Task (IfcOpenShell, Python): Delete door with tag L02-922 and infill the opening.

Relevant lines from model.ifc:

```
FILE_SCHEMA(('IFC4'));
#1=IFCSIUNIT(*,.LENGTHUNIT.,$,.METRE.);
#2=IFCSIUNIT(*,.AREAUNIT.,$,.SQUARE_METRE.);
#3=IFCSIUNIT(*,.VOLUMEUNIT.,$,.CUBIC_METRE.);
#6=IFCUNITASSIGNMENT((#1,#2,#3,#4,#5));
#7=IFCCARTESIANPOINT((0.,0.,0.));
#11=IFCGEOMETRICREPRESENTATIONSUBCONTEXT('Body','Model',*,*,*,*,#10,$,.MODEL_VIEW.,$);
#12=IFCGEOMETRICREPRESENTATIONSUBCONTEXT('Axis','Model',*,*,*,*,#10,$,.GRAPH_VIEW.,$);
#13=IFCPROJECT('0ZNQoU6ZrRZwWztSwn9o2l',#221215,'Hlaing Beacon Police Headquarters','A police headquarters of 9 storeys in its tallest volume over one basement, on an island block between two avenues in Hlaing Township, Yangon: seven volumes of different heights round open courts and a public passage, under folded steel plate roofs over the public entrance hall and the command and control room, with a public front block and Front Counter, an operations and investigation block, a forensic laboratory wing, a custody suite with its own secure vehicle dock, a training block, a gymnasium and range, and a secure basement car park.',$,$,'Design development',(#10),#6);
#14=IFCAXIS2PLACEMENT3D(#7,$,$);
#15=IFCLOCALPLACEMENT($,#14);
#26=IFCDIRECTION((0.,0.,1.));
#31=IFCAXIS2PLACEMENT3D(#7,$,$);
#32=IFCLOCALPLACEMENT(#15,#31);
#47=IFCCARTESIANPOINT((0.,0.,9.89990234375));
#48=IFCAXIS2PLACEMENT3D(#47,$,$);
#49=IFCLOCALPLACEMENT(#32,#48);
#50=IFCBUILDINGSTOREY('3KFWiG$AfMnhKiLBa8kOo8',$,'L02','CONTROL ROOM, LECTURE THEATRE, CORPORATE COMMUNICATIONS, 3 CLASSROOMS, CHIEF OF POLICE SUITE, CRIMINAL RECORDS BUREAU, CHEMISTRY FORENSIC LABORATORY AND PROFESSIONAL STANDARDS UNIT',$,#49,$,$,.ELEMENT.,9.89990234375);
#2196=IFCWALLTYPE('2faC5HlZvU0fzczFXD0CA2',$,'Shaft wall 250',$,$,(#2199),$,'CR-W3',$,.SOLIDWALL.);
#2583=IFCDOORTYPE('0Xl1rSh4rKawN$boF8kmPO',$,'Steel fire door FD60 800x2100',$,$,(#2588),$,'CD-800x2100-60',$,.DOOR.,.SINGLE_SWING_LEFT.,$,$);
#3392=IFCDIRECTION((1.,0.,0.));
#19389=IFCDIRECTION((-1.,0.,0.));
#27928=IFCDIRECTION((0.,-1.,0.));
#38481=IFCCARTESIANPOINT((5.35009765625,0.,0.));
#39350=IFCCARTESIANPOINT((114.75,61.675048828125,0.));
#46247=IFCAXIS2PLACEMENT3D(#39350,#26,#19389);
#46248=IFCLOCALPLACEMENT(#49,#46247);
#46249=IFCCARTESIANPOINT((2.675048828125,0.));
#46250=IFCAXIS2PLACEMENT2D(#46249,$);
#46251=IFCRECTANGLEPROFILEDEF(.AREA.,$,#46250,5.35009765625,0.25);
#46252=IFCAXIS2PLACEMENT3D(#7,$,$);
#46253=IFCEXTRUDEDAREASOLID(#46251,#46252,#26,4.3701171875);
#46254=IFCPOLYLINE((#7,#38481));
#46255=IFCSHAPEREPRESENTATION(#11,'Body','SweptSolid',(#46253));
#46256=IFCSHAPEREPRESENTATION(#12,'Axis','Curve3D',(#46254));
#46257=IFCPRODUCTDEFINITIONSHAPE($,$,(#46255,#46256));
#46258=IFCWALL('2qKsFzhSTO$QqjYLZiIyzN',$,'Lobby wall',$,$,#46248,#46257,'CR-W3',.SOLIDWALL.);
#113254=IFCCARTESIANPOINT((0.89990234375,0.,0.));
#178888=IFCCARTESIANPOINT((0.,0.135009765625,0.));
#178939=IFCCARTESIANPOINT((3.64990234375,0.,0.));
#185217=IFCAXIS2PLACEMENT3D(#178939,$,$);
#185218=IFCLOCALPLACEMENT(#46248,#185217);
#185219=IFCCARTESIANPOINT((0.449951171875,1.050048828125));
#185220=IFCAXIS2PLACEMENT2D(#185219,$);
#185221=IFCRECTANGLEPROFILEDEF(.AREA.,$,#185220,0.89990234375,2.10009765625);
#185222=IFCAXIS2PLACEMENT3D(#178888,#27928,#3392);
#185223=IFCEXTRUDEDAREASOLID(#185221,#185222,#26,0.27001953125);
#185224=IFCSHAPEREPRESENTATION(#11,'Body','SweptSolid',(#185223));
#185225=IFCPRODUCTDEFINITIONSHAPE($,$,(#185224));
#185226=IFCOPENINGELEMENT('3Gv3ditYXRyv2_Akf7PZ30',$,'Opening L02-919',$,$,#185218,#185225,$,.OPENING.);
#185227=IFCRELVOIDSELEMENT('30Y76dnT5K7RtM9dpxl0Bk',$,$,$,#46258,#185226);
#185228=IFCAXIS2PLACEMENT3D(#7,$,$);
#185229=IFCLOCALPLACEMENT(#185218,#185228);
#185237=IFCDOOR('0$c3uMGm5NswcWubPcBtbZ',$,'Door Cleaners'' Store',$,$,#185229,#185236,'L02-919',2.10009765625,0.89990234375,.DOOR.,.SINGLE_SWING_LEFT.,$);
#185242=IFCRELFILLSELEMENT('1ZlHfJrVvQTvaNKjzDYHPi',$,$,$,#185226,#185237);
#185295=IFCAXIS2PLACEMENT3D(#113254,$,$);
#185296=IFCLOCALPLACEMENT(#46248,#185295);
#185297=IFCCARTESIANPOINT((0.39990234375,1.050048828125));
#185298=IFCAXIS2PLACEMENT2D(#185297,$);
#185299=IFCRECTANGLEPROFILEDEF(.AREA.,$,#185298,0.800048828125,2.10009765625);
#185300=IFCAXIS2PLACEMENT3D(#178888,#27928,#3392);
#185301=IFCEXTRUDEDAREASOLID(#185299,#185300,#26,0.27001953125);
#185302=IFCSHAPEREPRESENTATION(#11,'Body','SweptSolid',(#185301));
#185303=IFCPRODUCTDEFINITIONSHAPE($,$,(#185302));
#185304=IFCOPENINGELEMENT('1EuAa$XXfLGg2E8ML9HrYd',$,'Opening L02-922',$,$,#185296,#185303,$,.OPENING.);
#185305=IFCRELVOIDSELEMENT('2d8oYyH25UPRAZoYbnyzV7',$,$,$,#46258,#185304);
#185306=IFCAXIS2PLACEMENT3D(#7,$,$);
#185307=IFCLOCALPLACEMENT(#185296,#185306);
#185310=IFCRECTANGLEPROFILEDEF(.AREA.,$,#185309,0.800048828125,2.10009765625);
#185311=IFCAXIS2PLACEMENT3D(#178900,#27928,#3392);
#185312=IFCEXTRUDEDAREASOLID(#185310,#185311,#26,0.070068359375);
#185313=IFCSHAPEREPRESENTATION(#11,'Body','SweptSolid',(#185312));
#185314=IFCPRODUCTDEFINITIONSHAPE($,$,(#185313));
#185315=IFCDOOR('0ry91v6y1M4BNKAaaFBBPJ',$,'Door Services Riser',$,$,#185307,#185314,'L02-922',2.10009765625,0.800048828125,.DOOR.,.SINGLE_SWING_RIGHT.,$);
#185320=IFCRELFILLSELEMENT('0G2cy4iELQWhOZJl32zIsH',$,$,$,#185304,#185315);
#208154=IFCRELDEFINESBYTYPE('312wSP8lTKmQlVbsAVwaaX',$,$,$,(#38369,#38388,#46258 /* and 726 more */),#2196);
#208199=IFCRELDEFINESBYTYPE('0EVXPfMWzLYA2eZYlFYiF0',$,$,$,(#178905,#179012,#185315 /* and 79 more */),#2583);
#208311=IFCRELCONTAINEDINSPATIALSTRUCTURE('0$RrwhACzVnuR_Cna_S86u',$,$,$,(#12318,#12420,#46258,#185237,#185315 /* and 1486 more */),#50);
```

```python
import ifcopenshell
import ifcopenshell.api.feature
import ifcopenshell.api.root
import ifcopenshell.geom
import ifcopenshell.util.shape

model = ifcopenshell.open("model.ifc")
settings = ifcopenshell.geom.settings()


def volume(element):
    """Net volume in cubic metres, openings subtracted."""
    shape = ifcopenshell.geom.create_shape(settings, element)
    return ifcopenshell.util.shape.get_volume(shape.geometry)


door = model.by_id(185315)
opening = door.FillsVoids[0].RelatingOpeningElement
wall = opening.VoidsElements[0].RelatingBuildingElement
before = volume(wall)

ifcopenshell.api.root.remove_product(model, product=door)
ifcopenshell.api.feature.remove_feature(model, feature=opening)

after = volume(wall)

print(f"wall volume {before:.3f} -> {after:.3f} m3")

model.write("model-out.ifc")
```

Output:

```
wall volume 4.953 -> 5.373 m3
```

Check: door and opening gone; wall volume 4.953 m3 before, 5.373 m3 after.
